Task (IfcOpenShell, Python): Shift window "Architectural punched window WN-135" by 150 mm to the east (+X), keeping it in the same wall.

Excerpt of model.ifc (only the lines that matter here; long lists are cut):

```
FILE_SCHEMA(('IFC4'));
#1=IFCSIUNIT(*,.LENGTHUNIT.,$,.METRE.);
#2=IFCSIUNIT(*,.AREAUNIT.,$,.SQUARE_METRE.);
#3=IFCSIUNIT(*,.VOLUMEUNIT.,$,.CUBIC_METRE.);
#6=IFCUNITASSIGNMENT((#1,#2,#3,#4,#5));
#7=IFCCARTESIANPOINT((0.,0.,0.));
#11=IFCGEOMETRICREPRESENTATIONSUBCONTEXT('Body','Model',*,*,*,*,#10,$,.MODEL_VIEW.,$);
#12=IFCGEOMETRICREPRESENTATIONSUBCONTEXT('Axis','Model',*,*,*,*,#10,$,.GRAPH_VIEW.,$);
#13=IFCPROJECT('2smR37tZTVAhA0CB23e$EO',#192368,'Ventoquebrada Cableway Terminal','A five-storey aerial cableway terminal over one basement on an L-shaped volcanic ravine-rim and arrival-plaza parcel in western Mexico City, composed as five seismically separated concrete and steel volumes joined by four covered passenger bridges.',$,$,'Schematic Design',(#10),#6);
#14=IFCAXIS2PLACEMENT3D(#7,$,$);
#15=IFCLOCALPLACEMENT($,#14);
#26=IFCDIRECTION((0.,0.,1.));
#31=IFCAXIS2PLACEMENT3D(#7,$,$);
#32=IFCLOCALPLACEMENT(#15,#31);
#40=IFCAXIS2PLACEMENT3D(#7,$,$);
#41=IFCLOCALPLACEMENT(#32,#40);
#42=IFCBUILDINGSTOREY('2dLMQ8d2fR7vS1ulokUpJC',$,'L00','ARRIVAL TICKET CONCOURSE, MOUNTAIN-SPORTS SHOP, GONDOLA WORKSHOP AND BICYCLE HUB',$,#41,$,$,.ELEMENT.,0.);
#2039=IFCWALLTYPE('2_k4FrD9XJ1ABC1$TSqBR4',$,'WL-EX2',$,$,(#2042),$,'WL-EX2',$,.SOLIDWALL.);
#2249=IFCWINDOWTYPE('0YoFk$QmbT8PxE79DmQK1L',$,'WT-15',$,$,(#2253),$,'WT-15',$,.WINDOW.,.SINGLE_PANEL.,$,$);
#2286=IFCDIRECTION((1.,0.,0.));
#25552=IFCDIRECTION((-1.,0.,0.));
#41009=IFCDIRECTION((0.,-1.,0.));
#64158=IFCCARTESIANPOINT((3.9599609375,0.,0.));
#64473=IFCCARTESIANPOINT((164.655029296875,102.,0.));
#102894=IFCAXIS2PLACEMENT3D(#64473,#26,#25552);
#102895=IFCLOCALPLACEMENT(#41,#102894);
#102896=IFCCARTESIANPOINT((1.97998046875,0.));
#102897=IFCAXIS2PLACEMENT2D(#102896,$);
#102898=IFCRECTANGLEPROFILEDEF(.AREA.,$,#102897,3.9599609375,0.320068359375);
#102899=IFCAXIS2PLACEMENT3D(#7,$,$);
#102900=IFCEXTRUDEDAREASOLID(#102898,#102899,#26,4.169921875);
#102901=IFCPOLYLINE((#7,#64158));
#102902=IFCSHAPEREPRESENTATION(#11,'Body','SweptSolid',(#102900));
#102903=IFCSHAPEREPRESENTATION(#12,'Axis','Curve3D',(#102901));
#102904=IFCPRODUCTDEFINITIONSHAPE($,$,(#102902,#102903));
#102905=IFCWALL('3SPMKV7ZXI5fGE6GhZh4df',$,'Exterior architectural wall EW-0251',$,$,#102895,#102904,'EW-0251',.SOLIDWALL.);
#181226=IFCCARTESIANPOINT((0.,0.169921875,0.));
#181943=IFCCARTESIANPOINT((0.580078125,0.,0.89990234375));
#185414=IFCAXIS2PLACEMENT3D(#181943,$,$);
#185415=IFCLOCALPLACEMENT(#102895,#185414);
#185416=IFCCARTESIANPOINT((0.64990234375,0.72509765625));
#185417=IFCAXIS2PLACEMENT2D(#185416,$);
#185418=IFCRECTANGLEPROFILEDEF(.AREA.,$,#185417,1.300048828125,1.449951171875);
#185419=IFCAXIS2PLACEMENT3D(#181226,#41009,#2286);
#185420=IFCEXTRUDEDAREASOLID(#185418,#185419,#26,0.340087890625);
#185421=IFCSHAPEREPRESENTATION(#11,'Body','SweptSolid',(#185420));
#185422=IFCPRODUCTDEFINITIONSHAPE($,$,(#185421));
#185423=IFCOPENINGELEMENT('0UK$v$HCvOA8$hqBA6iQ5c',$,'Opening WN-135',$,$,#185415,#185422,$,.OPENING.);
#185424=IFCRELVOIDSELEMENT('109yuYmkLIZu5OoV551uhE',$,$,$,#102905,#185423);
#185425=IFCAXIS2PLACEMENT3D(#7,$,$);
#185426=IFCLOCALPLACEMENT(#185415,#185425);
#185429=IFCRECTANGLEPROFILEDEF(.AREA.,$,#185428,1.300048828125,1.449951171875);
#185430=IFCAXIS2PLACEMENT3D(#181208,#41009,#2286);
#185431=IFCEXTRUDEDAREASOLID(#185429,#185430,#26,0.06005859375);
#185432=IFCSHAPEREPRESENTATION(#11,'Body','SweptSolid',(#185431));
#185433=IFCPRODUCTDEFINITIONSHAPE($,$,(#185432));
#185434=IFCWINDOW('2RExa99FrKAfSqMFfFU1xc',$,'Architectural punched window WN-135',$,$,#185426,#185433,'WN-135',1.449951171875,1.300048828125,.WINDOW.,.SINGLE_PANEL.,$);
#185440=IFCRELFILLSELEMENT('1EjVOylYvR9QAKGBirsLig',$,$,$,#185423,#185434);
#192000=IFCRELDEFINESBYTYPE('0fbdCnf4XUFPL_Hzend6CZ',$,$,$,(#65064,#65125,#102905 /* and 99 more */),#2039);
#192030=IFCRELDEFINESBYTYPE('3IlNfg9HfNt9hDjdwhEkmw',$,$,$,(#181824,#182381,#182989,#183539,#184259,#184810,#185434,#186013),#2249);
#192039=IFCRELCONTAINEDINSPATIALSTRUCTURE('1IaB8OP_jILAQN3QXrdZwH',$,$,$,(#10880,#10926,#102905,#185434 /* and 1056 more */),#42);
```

```python
import ifcopenshell
import ifcopenshell.api.geometry
import ifcopenshell.util.placement
import ifcopenshell.util.unit

model = ifcopenshell.open("model.ifc")
unit_scale = ifcopenshell.util.unit.calculate_unit_scale(model)

window = model.by_id(185434)
opening = window.FillsVoids[0].RelatingOpeningElement
wall = opening.VoidsElements[0].RelatingBuildingElement

wall_matrix = ifcopenshell.util.placement.get_local_placement(wall.ObjectPlacement)
shift = wall_matrix[:3, 0] * -0.15 / unit_scale
before = ifcopenshell.util.placement.get_local_placement(window.ObjectPlacement)[:3, 3].copy()

# The window is placed relative to its opening, so it follows when the opening moves.
matrix = ifcopenshell.util.placement.get_local_placement(opening.ObjectPlacement)
matrix[:3, 3] += shift
ifcopenshell.api.geometry.edit_object_placement(
    model, product=opening, matrix=matrix, is_si=False, should_transform_children=True
)

after = ifcopenshell.util.placement.get_local_placement(window.ObjectPlacement)[:3, 3]
print("window moved by", (after - before).round(3) + 0.0)

model.write("model-out.ifc")
```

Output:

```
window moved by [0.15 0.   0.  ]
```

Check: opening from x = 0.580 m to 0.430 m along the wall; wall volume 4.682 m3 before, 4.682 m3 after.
